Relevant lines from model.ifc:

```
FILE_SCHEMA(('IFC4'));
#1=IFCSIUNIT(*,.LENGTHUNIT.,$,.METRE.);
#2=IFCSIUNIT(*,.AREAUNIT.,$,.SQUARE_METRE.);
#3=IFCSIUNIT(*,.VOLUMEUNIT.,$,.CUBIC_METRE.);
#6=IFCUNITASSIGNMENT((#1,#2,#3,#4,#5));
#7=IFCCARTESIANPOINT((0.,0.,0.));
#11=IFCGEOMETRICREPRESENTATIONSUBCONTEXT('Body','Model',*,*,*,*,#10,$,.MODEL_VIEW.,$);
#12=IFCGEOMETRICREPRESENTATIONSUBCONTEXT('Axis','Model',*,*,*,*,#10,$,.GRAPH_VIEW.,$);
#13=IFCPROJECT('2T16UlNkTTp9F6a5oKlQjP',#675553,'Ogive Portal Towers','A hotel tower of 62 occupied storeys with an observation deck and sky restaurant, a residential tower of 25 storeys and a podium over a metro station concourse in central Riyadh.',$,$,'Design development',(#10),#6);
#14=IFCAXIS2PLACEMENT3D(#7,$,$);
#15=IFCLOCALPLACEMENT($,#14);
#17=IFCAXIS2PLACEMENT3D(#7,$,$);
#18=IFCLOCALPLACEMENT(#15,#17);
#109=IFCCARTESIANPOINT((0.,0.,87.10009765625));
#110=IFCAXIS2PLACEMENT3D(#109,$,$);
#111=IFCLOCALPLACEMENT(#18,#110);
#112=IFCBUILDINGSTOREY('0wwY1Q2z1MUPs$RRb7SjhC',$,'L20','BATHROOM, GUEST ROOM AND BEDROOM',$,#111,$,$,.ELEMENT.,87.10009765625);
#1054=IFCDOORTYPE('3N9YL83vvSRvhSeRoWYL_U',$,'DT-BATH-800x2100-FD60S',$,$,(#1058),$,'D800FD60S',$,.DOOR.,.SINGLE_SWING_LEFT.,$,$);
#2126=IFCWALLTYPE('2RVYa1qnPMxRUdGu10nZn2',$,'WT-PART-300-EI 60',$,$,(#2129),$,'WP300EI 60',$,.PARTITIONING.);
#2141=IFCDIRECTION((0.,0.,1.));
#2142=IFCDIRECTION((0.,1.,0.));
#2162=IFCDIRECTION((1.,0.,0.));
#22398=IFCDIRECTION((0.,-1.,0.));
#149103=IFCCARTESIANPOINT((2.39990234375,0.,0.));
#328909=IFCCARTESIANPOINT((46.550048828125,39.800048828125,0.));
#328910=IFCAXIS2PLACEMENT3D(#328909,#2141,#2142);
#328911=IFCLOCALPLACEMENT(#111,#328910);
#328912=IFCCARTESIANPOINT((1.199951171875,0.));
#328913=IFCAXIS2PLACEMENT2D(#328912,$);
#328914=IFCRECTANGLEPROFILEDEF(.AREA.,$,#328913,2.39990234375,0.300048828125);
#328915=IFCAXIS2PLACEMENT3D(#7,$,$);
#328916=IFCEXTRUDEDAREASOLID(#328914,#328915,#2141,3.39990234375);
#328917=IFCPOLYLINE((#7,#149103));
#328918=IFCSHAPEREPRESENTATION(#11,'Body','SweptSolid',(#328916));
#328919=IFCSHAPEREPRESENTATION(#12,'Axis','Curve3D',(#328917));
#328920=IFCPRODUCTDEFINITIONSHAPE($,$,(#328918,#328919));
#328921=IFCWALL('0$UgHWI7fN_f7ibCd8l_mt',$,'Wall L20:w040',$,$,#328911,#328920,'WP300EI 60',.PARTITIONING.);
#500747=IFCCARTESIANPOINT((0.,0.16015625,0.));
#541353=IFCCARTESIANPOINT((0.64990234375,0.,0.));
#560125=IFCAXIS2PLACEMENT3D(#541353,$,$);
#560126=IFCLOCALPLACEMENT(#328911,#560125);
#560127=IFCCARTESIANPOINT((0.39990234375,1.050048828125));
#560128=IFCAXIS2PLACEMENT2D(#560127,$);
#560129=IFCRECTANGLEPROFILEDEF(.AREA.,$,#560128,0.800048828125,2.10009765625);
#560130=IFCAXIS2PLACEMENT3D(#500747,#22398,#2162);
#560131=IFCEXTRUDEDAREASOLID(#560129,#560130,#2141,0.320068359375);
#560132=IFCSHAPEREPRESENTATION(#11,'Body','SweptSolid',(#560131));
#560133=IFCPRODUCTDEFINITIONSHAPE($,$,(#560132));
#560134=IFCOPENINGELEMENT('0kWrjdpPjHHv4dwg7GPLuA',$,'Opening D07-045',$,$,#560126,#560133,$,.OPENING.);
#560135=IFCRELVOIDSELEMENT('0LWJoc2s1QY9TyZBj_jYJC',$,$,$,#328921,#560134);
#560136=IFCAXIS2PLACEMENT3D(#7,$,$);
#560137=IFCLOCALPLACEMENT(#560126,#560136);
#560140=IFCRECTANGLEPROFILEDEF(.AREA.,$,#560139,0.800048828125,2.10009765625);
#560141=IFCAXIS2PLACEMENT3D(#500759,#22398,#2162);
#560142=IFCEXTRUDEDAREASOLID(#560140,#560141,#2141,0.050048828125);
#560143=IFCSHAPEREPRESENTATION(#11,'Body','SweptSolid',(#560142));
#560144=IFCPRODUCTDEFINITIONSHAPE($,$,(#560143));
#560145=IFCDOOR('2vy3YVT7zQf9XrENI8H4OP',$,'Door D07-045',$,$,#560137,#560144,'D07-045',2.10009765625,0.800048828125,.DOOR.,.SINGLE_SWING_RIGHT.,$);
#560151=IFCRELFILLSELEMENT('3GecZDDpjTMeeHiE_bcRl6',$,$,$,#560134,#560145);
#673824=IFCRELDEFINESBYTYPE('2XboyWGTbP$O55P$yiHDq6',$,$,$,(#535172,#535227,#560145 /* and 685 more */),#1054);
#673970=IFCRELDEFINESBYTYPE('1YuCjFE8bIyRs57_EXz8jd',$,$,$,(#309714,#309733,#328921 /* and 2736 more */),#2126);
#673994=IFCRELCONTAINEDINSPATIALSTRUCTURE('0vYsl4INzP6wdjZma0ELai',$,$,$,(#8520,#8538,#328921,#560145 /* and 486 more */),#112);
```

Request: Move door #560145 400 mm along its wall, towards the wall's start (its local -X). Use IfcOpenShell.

```python
import ifcopenshell
import ifcopenshell.api.geometry
import ifcopenshell.util.placement

model = ifcopenshell.open("model.ifc")

door = model.by_id(560145)
opening = door.FillsVoids[0].RelatingOpeningElement
wall = opening.VoidsElements[0].RelatingBuildingElement

wall_matrix = ifcopenshell.util.placement.get_local_placement(wall.ObjectPlacement)
shift = wall_matrix[:3, 0] * -0.4
before = ifcopenshell.util.placement.get_local_placement(door.ObjectPlacement)[:3, 3].copy()

# The door is placed relative to its opening, so it follows when the opening moves.
matrix = ifcopenshell.util.placement.get_local_placement(opening.ObjectPlacement)
matrix[:3, 3] += shift
ifcopenshell.api.geometry.edit_object_placement(
    model, product=opening, matrix=matrix, is_si=False, should_transform_children=True
)

after = ifcopenshell.util.placement.get_local_placement(door.ObjectPlacement)[:3, 3]
print("door moved by", (after - before).round(3) + 0.0)

model.write("model_updated.ifc")
```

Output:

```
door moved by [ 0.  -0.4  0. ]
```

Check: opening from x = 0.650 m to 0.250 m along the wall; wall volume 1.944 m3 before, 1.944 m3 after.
